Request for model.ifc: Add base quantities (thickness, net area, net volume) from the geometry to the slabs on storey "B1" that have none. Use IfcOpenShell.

First a look at what the model holds.

```python
import ifcopenshell
import ifcopenshell.util.element
import ifcopenshell.util.unit

model = ifcopenshell.open("model.ifc")
print(model.schema)
for unit_type in ("LENGTHUNIT", "AREAUNIT", "VOLUMEUNIT"):
    print(unit_type, ifcopenshell.util.unit.calculate_unit_scale(model, unit_type))
storey = next(s for s in model.by_type("IfcBuildingStorey") if s.Name == "B1")
slabs = [e for e in ifcopenshell.util.element.get_decomposition(storey) if e.is_a("IfcSlab")]
for e in sorted(slabs, key=lambda e: e.id()):
    print(e.id(), e.is_a(), e.Name, list(ifcopenshell.util.element.get_psets(e, qtos_only=True)), sep=" | ")
```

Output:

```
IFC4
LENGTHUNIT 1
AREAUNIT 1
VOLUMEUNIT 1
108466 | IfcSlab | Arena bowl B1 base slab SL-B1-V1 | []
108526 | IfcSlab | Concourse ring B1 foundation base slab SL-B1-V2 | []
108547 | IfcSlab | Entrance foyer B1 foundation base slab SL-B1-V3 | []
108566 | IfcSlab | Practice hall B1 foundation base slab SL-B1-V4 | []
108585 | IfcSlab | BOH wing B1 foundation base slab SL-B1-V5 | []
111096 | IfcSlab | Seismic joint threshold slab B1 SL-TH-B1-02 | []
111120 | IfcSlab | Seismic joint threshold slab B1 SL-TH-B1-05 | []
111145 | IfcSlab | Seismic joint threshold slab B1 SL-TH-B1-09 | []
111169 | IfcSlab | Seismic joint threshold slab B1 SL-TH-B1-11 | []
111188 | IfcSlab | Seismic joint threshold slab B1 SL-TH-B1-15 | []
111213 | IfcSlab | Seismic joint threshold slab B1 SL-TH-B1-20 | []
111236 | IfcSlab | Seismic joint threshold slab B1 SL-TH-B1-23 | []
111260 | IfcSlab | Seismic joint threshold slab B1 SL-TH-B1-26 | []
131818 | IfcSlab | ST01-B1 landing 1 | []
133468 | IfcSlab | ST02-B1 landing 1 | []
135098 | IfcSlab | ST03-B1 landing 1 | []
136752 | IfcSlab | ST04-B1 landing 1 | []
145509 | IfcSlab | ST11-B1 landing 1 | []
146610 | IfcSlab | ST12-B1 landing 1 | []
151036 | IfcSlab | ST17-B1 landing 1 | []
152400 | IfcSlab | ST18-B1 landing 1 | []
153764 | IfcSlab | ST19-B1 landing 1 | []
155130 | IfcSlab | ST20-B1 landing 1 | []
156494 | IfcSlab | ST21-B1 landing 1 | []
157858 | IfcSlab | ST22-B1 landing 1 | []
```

```python
import ifcopenshell
import ifcopenshell.api.pset
import ifcopenshell.geom
import ifcopenshell.util.element
import ifcopenshell.util.shape
import ifcopenshell.util.unit

model = ifcopenshell.open("model.ifc")
unit_scale = ifcopenshell.util.unit.calculate_unit_scale(model)
area_scale = ifcopenshell.util.unit.calculate_unit_scale(model, "AREAUNIT")
volume_scale = ifcopenshell.util.unit.calculate_unit_scale(model, "VOLUMEUNIT")
settings = ifcopenshell.geom.settings()

storey = next(s for s in model.by_type("IfcBuildingStorey") if s.Name == "B1")
slabs = [e for e in ifcopenshell.util.element.get_decomposition(storey) if e.is_a("IfcSlab")]

for e in sorted(slabs, key=lambda e: e.id()):
    if ifcopenshell.util.element.get_psets(e, qtos_only=True, should_inherit=False):
        continue
    # Geometry comes back in metres, in the element's own axes.
    shape = ifcopenshell.geom.create_shape(settings, e)
    values = {
        "Width": ifcopenshell.util.shape.get_z(shape.geometry) / unit_scale,
        "NetArea": ifcopenshell.util.shape.get_footprint_area(shape.geometry) / area_scale,
        "NetVolume": ifcopenshell.util.shape.get_volume(shape.geometry) / volume_scale,
    }
    qto = ifcopenshell.api.pset.add_qto(model, product=e, name="Qto_SlabBaseQuantities")
    ifcopenshell.api.pset.edit_qto(model, qto=qto, properties=values)
    print(e.id(), {k: round(v, 3) for k, v in values.items()})

model.write("model_updated.ifc")
```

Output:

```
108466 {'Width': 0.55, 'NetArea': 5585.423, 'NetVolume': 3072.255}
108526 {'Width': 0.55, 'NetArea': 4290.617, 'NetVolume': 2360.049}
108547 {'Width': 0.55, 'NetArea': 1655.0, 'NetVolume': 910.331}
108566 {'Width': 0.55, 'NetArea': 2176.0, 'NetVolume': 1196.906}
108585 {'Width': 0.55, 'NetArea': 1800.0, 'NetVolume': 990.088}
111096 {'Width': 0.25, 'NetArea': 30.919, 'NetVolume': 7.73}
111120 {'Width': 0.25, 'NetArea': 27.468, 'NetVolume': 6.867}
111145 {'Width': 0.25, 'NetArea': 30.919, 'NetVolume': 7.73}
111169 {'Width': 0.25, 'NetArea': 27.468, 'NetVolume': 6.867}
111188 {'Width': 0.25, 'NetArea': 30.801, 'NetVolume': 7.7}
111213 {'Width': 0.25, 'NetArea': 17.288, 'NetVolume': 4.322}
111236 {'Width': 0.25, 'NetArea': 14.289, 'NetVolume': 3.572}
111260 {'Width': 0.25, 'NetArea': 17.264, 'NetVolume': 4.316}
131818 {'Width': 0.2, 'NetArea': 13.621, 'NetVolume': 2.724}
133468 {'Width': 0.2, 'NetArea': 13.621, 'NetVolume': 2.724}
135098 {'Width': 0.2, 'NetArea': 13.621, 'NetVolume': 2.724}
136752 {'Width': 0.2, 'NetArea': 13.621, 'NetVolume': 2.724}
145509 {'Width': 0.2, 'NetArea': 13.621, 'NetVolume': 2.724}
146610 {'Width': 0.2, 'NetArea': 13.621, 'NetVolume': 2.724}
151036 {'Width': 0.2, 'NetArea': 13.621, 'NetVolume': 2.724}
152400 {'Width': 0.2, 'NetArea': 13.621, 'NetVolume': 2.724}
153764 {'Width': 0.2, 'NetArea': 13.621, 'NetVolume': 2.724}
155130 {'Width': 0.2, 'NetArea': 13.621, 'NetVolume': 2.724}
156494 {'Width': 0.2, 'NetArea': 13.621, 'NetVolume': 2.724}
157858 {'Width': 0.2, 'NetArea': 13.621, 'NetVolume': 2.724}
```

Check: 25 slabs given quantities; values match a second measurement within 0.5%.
